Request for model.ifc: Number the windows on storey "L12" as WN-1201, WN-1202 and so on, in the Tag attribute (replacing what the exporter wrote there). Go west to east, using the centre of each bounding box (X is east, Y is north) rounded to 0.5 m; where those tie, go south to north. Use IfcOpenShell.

First a look at what the model holds.

```python
import ifcopenshell
import ifcopenshell.util.element
import ifcopenshell.util.placement

model = ifcopenshell.open("model.ifc")
print(model.schema)
storey = next(s for s in model.by_type("IfcBuildingStorey") if s.Name == "L12")
windows = [e for e in ifcopenshell.util.element.get_decomposition(storey) if e.is_a("IfcWindow")]
for e in sorted(windows, key=lambda e: e.id()):
    origin = ifcopenshell.util.placement.get_local_placement(e.ObjectPlacement)[:3, 3]
    print(e.id(), e.Tag, e.Name, origin.round(2) + 0.0, sep=" | ")
```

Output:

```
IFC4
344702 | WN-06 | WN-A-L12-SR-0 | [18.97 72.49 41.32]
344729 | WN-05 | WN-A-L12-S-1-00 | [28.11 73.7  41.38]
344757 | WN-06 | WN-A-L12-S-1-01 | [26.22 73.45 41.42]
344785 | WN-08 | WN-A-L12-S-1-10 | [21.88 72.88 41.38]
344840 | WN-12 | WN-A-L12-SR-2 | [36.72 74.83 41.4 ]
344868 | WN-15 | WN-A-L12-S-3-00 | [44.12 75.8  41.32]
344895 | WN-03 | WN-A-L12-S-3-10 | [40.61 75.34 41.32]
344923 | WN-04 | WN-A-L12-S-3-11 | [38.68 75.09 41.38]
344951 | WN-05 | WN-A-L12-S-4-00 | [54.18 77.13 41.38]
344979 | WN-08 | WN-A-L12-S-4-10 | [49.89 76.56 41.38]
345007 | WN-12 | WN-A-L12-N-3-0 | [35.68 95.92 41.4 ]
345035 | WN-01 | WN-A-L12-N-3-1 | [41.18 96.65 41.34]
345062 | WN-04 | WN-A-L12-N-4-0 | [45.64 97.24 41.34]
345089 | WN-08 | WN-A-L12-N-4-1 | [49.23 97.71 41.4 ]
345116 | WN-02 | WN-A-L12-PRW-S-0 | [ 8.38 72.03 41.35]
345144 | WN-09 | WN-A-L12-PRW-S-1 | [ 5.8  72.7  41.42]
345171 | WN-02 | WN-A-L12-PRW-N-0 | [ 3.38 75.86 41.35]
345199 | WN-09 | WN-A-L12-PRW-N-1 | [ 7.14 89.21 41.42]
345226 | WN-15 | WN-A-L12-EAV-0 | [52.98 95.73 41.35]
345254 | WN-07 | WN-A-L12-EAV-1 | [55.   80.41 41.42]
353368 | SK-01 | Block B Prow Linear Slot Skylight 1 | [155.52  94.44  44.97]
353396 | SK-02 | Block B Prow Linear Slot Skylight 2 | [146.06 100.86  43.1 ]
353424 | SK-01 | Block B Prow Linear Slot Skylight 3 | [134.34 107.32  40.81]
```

```python
import ifcopenshell
import ifcopenshell.geom
import ifcopenshell.util.element
import ifcopenshell.util.shape

model = ifcopenshell.open("model.ifc")
settings = ifcopenshell.geom.settings()
settings.set("use-world-coords", True)


def centre(element):
    shape = ifcopenshell.geom.create_shape(settings, element)
    return ifcopenshell.util.shape.get_bbox_centroid(shape.geometry)


storey = next(s for s in model.by_type("IfcBuildingStorey") if s.Name == "L12")
windows = [e for e in ifcopenshell.util.element.get_decomposition(storey) if e.is_a("IfcWindow")]

# Insertion points can sit at a corner or the storey origin, so sort by the geometry (in metres).
centres = {e: centre(e) for e in windows}
windows.sort(key=lambda e: (round(centres[e][0] / 0.5), centres[e][1]))

for i, e in enumerate(windows, start=1):
    number = f"WN-12{i:02d}"
    e.Tag = number
    print(e.id(), number)

model.write("model-out.ifc")
```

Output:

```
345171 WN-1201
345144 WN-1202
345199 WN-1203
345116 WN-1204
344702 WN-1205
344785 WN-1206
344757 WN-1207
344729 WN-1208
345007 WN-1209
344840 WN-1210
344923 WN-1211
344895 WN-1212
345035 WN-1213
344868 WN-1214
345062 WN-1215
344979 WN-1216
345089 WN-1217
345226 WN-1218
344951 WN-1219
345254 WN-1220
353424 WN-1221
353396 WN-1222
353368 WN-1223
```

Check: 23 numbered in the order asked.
